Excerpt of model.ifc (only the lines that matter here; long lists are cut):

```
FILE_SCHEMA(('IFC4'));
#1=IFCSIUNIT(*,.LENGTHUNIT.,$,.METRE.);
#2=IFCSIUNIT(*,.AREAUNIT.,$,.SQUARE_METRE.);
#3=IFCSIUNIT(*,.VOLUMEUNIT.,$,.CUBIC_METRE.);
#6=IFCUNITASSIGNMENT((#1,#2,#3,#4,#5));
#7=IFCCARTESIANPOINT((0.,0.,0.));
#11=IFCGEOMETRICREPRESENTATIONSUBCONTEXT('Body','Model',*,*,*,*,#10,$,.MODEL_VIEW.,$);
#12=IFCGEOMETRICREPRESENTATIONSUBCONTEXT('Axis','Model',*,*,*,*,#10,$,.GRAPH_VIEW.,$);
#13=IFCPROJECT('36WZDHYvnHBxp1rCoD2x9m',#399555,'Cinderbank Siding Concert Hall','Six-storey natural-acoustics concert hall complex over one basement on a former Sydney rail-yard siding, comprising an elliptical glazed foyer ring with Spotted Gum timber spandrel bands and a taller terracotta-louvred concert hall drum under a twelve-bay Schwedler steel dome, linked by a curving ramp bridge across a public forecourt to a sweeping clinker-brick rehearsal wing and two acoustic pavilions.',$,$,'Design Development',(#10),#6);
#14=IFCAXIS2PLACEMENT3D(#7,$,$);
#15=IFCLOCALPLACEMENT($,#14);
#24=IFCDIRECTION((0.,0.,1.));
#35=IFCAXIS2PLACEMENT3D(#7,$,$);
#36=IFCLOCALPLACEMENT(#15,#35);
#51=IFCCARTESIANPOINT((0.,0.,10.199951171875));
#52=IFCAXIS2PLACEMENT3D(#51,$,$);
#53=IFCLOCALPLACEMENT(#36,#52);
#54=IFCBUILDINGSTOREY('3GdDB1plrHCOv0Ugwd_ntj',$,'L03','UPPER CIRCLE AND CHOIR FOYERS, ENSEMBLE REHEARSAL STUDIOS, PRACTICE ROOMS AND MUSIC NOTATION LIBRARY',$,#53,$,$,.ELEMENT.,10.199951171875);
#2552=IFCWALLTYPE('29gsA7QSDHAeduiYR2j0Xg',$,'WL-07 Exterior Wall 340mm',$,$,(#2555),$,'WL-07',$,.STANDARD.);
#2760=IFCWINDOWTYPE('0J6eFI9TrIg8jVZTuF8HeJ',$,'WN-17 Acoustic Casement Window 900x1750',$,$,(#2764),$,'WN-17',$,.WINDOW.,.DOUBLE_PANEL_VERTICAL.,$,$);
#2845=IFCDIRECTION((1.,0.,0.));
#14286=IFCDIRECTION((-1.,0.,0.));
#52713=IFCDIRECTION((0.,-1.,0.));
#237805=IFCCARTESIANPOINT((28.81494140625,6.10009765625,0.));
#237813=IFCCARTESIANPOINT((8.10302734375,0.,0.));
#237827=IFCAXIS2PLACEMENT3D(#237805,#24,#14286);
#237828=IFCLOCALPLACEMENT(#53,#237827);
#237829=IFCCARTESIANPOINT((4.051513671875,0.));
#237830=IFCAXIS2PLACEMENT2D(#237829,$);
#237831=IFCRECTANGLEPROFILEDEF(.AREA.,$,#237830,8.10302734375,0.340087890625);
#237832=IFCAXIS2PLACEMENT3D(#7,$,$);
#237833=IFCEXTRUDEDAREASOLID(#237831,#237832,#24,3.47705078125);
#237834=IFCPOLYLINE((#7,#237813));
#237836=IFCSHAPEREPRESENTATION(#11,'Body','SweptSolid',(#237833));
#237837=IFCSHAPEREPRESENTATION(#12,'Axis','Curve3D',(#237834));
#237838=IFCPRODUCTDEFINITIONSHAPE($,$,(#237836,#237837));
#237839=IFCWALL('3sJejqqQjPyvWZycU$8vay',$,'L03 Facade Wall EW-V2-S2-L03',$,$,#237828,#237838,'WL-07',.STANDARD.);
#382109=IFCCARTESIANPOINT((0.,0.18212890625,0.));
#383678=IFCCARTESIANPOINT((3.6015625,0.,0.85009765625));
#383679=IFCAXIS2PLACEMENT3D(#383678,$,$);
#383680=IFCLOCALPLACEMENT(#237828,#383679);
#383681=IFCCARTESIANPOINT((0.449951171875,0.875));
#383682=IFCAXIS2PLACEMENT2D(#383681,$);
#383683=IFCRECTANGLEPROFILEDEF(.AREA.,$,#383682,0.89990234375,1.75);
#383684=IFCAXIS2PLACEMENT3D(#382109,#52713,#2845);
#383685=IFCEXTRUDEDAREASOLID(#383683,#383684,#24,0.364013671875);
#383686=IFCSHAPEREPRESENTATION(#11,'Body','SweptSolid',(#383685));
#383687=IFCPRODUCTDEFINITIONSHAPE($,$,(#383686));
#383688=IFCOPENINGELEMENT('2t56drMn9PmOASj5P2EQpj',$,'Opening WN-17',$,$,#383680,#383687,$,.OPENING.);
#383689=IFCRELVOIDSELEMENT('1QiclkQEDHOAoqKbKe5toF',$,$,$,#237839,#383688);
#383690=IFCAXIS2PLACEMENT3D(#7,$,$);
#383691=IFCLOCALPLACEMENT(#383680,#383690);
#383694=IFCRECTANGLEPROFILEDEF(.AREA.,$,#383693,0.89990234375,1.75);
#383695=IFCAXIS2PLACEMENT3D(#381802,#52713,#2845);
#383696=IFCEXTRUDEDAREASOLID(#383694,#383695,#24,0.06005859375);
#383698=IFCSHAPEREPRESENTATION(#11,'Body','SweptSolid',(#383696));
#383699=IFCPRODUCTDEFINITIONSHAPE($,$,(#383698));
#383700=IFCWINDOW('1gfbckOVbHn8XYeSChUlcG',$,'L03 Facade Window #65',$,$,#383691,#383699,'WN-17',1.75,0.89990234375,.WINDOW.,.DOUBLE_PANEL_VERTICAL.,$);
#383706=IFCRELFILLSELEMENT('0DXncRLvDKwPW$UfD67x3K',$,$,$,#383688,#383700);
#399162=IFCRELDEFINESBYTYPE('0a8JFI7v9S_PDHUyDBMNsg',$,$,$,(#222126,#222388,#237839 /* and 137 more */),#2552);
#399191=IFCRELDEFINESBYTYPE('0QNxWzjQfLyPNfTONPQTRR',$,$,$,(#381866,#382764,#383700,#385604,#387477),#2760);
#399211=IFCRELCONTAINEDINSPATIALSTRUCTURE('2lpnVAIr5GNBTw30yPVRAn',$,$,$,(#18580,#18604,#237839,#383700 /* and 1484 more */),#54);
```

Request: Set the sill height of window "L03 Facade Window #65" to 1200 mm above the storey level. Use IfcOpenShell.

```python
import numpy as np
import ifcopenshell
import ifcopenshell.api.geometry
import ifcopenshell.geom
import ifcopenshell.util.element
import ifcopenshell.util.placement
import ifcopenshell.util.shape
import ifcopenshell.util.unit

model = ifcopenshell.open("model.ifc")
unit_scale = ifcopenshell.util.unit.calculate_unit_scale(model)

window = model.by_id(383700)
opening = window.FillsVoids[0].RelatingOpeningElement
storey = ifcopenshell.util.element.get_container(window, ifc_class="IfcBuildingStorey")
level = ifcopenshell.util.placement.get_local_placement(storey.ObjectPlacement)[2, 3]

# The opening's origin need not be at the sill, so measure its lowest point.
shape = ifcopenshell.geom.create_shape(ifcopenshell.geom.settings(), opening)
bottom = ifcopenshell.util.shape.get_shape_bottom_elevation(shape, shape.geometry) / unit_scale
dz = level + 1.2 - bottom

shift = np.array([0.0, 0.0, dz])
# The window is placed relative to its opening, so it follows when the opening moves.
matrix = ifcopenshell.util.placement.get_local_placement(opening.ObjectPlacement)
matrix[:3, 3] += shift
ifcopenshell.api.geometry.edit_object_placement(
    model, product=opening, matrix=matrix, is_si=False, should_transform_children=True
)

print(f"moved by {dz * unit_scale:+.3f} m")

model.write("model_updated.ifc")
```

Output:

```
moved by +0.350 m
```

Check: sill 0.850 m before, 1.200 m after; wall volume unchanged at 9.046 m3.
